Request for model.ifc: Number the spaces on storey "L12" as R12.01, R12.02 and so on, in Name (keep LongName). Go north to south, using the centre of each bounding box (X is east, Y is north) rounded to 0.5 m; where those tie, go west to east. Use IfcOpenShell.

First a look at what the model holds.

```python
import ifcopenshell
import ifcopenshell.util.element
import ifcopenshell.util.placement

model = ifcopenshell.open("model.ifc")
print(model.schema)
storey = next(s for s in model.by_type("IfcBuildingStorey") if s.Name == "L12")
spaces = [e for e in ifcopenshell.util.element.get_decomposition(storey) if e.is_a("IfcSpace")]
for e in sorted(spaces, key=lambda e: e.id()):
    origin = ifcopenshell.util.placement.get_local_placement(e.ObjectPlacement)[:3, 3]
    print(e.id(), e.Name, e.LongName, origin.round(2) + 0.0, sep=" | ")
```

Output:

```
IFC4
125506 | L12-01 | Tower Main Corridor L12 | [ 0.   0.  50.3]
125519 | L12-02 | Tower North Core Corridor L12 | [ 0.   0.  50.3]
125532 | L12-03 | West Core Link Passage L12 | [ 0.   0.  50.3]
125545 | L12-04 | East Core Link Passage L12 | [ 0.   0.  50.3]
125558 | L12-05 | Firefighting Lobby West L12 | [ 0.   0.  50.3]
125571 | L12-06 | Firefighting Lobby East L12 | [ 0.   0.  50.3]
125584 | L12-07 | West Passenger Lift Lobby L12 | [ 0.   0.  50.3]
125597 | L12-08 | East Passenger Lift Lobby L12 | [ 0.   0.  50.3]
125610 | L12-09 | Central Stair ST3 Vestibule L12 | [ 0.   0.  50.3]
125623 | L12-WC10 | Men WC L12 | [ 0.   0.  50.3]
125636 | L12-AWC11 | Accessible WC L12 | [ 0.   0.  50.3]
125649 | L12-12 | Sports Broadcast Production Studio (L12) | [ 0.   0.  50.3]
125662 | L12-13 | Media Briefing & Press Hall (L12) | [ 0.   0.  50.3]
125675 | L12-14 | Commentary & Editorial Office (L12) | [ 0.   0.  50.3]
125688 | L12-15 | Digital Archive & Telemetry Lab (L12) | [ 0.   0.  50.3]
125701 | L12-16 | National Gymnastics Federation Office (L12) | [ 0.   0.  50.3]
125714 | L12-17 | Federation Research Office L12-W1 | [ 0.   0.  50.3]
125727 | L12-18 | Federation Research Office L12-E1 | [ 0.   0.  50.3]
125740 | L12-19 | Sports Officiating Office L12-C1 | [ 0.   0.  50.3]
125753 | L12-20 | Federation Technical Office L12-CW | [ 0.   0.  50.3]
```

```python
import ifcopenshell
import ifcopenshell.geom
import ifcopenshell.util.element
import ifcopenshell.util.shape

model = ifcopenshell.open("model.ifc")
settings = ifcopenshell.geom.settings()
settings.set("use-world-coords", True)


def centre(element):
    shape = ifcopenshell.geom.create_shape(settings, element)
    return ifcopenshell.util.shape.get_bbox_centroid(shape.geometry)


storey = next(s for s in model.by_type("IfcBuildingStorey") if s.Name == "L12")
spaces = [e for e in ifcopenshell.util.element.get_decomposition(storey) if e.is_a("IfcSpace")]

# Insertion points can sit at a corner or the storey origin, so sort by the geometry (in metres).
centres = {e: centre(e) for e in spaces}
spaces.sort(key=lambda e: (-round(centres[e][1] / 0.5), centres[e][0]))

for i, e in enumerate(spaces, start=1):
    number = f"R12.{i:02d}"
    e.Name = number
    print(e.id(), number)

model.write("model_edited.ifc")
```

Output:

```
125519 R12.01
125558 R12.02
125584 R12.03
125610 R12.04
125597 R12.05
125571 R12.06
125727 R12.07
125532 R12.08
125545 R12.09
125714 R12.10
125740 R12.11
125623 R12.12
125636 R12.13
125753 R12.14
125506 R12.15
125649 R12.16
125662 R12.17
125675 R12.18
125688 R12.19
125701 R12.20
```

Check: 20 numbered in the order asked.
